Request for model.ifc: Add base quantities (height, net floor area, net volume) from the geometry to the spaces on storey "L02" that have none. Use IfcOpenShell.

First a look at what the model holds.

```python
import ifcopenshell
import ifcopenshell.util.element
import ifcopenshell.util.unit

model = ifcopenshell.open("model.ifc")
print(model.schema)
for unit_type in ("LENGTHUNIT", "AREAUNIT", "VOLUMEUNIT"):
    print(unit_type, ifcopenshell.util.unit.calculate_unit_scale(model, unit_type))
storey = next(s for s in model.by_type("IfcBuildingStorey") if s.Name == "L02")
spaces = [e for e in ifcopenshell.util.element.get_decomposition(storey) if e.is_a("IfcSpace")]
for e in sorted(spaces, key=lambda e: e.id()):
    print(e.id(), e.is_a(), e.Name, list(ifcopenshell.util.element.get_psets(e, qtos_only=True)), sep=" | ")
```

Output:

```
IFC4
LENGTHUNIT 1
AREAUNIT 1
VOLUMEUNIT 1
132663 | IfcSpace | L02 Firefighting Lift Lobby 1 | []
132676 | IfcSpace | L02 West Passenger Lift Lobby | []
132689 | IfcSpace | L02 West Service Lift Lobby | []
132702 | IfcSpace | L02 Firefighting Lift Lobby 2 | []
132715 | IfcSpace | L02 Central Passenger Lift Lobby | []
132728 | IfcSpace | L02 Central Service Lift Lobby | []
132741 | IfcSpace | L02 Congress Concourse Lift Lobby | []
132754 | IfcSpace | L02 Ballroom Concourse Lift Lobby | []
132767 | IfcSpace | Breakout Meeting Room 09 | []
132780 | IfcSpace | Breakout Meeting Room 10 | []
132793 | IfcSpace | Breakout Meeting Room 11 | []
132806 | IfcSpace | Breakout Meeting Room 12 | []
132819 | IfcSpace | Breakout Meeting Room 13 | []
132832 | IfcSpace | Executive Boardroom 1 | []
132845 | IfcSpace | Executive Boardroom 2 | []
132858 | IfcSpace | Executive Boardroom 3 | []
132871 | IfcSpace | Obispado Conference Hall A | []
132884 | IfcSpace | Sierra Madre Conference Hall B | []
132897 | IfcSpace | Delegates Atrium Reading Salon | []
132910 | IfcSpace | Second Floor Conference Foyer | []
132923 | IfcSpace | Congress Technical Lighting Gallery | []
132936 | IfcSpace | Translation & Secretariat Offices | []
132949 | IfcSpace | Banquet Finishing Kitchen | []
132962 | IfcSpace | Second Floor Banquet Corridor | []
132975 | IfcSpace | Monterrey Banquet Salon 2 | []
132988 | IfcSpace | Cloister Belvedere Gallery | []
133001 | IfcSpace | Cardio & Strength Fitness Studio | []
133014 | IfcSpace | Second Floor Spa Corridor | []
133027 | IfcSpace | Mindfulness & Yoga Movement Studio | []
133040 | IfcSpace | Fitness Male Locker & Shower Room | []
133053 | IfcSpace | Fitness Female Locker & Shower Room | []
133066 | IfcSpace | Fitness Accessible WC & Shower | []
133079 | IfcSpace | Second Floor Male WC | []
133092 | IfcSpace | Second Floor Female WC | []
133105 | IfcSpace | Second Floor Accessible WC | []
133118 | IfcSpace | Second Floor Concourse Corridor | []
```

```python
import ifcopenshell
import ifcopenshell.api.pset
import ifcopenshell.geom
import ifcopenshell.util.element
import ifcopenshell.util.shape
import ifcopenshell.util.unit

model = ifcopenshell.open("model.ifc")
unit_scale = ifcopenshell.util.unit.calculate_unit_scale(model)
area_scale = ifcopenshell.util.unit.calculate_unit_scale(model, "AREAUNIT")
volume_scale = ifcopenshell.util.unit.calculate_unit_scale(model, "VOLUMEUNIT")
settings = ifcopenshell.geom.settings()

storey = next(s for s in model.by_type("IfcBuildingStorey") if s.Name == "L02")
spaces = [e for e in ifcopenshell.util.element.get_decomposition(storey) if e.is_a("IfcSpace")]

for e in sorted(spaces, key=lambda e: e.id()):
    if ifcopenshell.util.element.get_psets(e, qtos_only=True, should_inherit=False):
        continue
    # Geometry comes back in metres, in the element's own axes.
    shape = ifcopenshell.geom.create_shape(settings, e)
    values = {
        "Height": ifcopenshell.util.shape.get_z(shape.geometry) / unit_scale,
        "NetFloorArea": ifcopenshell.util.shape.get_footprint_area(shape.geometry) / area_scale,
        "NetVolume": ifcopenshell.util.shape.get_volume(shape.geometry) / volume_scale,
    }
    qto = ifcopenshell.api.pset.add_qto(model, product=e, name="Qto_SpaceBaseQuantities")
    ifcopenshell.api.pset.edit_qto(model, qto=qto, properties=values)
    print(e.id(), {k: round(v, 3) for k, v in values.items()})

model.write("model-out.ifc")
```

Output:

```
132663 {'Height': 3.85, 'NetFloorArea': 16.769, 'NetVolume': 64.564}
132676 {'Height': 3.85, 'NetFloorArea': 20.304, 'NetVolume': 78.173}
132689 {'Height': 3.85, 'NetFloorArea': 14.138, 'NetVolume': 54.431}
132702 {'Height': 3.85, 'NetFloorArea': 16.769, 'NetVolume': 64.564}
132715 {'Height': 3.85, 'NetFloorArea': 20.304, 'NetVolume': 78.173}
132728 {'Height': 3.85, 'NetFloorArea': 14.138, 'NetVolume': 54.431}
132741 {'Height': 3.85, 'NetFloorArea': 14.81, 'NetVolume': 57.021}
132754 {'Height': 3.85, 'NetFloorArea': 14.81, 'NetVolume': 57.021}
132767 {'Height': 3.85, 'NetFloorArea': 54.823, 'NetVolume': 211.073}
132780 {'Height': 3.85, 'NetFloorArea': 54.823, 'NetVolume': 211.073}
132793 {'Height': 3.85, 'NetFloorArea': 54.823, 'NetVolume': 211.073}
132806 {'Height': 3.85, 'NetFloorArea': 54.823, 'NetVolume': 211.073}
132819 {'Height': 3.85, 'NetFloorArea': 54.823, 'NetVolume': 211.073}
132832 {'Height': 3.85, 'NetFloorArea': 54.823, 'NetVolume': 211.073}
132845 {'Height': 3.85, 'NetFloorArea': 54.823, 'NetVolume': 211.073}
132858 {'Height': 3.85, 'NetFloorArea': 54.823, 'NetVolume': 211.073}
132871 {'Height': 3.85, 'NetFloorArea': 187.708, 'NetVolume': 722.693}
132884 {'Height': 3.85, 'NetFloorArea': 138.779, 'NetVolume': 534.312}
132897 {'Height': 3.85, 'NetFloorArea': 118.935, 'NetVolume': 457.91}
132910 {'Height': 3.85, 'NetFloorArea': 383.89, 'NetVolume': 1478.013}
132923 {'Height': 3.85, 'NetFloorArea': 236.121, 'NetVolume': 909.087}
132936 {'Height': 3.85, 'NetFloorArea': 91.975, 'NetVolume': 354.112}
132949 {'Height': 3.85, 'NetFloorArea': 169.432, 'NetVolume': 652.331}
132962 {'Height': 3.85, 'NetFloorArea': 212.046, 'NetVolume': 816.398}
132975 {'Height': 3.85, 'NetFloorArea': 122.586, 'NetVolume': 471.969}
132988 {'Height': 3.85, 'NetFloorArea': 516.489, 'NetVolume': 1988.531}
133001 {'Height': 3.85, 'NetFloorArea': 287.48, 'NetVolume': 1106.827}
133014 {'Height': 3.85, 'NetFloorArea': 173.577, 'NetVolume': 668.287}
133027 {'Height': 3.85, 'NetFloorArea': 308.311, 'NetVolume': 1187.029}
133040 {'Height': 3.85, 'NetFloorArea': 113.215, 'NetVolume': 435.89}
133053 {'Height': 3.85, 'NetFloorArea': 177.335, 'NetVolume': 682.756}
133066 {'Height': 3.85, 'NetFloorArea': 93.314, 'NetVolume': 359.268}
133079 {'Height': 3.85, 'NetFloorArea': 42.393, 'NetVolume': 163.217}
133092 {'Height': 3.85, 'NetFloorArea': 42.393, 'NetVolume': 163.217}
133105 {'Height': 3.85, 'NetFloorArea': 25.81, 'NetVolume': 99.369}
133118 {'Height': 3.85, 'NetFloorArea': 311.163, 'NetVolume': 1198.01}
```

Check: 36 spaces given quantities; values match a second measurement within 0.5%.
